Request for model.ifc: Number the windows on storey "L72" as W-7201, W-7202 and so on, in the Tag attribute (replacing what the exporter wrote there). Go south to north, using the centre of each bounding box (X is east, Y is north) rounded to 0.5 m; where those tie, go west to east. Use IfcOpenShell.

First a look at what the model holds.

```python
import ifcopenshell
import ifcopenshell.util.element
import ifcopenshell.util.placement

model = ifcopenshell.open("model.ifc")
print(model.schema)
storey = next(s for s in model.by_type("IfcBuildingStorey") if s.Name == "L72")
windows = [e for e in ifcopenshell.util.element.get_decomposition(storey) if e.is_a("IfcWindow")]
for e in sorted(windows, key=lambda e: e.id()):
    origin = ifcopenshell.util.placement.get_local_placement(e.ObjectPlacement)[:3, 3]
    print(e.id(), e.Tag, e.Name, origin.round(2) + 0.0, sep=" | ")
```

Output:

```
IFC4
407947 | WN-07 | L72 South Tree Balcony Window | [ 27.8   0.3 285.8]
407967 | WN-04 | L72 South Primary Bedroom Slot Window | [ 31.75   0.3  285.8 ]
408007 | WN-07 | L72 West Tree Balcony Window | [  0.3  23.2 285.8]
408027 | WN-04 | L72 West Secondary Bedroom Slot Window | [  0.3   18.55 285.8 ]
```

```python
import ifcopenshell
import ifcopenshell.geom
import ifcopenshell.util.element
import ifcopenshell.util.shape

model = ifcopenshell.open("model.ifc")
settings = ifcopenshell.geom.settings()
settings.set("use-world-coords", True)


def centre(element):
    shape = ifcopenshell.geom.create_shape(settings, element)
    return ifcopenshell.util.shape.get_bbox_centroid(shape.geometry)


storey = next(s for s in model.by_type("IfcBuildingStorey") if s.Name == "L72")
windows = [e for e in ifcopenshell.util.element.get_decomposition(storey) if e.is_a("IfcWindow")]

# Insertion points can sit at a corner or the storey origin, so sort by the geometry (in metres).
centres = {e: centre(e) for e in windows}
windows.sort(key=lambda e: (round(centres[e][1] / 0.5), centres[e][0]))

for i, e in enumerate(windows, start=1):
    number = f"W-72{i:02d}"
    e.Tag = number
    print(e.id(), number)

model.write("model-out.ifc")
```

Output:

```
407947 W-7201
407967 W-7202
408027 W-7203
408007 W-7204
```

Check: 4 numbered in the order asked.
